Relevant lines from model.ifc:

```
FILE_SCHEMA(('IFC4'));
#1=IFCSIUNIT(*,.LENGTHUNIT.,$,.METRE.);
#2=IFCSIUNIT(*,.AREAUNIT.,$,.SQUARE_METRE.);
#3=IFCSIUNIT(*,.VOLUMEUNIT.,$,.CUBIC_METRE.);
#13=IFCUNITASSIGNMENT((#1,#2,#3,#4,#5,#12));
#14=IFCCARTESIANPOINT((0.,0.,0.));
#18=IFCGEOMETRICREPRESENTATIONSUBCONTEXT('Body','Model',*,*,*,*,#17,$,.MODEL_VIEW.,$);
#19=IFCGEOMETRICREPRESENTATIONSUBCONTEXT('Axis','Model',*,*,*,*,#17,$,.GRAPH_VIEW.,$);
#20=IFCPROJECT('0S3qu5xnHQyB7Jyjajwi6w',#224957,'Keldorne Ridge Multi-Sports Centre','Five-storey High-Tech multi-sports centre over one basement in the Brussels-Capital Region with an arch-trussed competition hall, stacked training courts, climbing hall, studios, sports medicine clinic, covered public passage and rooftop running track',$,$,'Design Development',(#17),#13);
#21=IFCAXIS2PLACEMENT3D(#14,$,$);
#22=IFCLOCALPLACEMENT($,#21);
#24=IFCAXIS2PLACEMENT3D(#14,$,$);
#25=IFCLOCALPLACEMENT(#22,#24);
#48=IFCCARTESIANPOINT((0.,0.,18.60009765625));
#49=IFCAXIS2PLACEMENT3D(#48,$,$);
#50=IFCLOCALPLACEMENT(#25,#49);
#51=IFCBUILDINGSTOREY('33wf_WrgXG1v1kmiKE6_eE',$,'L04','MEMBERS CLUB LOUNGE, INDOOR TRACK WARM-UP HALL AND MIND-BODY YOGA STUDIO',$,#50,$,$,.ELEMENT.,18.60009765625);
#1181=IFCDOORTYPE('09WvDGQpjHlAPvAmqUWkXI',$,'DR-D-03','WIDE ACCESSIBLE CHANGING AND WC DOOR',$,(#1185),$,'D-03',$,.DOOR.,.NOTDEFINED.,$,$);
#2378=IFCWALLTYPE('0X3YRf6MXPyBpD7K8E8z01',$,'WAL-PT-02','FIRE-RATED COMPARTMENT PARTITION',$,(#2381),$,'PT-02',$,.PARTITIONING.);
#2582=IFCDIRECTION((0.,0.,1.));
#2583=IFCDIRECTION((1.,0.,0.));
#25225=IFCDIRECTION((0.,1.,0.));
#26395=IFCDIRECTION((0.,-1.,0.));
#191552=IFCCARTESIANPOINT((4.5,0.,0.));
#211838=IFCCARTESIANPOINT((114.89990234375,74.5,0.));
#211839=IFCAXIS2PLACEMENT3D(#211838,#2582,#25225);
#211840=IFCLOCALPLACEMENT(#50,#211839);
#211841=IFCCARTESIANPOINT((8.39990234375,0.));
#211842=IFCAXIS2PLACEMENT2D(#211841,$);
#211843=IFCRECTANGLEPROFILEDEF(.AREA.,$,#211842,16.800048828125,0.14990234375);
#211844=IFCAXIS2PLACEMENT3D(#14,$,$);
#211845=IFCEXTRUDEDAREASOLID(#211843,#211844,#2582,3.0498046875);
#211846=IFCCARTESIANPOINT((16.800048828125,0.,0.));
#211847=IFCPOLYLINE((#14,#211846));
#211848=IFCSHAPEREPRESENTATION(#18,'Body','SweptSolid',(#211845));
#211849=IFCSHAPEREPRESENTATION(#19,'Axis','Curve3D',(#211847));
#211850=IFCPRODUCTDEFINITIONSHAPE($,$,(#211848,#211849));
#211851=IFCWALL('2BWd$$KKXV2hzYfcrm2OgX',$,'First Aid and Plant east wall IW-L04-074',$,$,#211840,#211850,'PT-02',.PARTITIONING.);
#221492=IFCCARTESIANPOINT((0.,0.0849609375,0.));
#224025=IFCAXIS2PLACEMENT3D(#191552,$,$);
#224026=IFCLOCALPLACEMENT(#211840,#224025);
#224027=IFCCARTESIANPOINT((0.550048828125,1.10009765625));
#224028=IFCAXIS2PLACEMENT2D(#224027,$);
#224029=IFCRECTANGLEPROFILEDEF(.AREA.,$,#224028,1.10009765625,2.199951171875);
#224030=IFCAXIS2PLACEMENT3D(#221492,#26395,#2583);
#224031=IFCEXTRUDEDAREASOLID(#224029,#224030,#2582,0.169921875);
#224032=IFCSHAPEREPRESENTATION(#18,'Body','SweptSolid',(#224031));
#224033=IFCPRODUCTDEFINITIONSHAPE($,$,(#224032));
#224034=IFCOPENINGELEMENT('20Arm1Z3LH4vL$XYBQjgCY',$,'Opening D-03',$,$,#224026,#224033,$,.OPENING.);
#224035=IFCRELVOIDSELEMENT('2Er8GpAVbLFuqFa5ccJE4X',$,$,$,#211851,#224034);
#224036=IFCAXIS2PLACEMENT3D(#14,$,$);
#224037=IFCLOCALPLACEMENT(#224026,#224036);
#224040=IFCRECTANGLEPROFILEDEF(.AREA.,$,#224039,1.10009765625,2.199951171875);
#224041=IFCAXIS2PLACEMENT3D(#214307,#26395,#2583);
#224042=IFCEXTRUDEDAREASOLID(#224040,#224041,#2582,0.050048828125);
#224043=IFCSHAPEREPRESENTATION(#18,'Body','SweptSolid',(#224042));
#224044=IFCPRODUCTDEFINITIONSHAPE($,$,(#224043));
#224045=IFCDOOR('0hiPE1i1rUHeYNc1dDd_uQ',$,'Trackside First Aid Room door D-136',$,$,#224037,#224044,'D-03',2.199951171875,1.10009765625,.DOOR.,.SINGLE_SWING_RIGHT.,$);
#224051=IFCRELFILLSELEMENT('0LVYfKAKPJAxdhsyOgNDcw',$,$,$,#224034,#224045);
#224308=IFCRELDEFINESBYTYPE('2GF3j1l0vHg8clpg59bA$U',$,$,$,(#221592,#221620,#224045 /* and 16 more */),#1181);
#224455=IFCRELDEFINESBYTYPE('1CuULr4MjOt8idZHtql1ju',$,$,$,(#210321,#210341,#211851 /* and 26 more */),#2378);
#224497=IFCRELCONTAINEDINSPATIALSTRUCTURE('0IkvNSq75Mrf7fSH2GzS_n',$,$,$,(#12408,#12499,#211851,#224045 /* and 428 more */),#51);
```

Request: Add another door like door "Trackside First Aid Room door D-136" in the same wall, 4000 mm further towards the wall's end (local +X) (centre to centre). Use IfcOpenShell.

```python
import ifcopenshell
import ifcopenshell.api.feature
import ifcopenshell.api.geometry
import ifcopenshell.api.root
import ifcopenshell.geom
import ifcopenshell.util.element
import ifcopenshell.util.placement
import ifcopenshell.util.shape

model = ifcopenshell.open("model.ifc")
settings = ifcopenshell.geom.settings()


def volume(element):
    """Net volume in cubic metres, openings subtracted."""
    shape = ifcopenshell.geom.create_shape(settings, element)
    return ifcopenshell.util.shape.get_volume(shape.geometry)


door = model.by_guid("0hiPE1i1rUHeYNc1dDd_uQ")
opening = door.FillsVoids[0].RelatingOpeningElement
wall = opening.VoidsElements[0].RelatingBuildingElement
before = volume(wall)
shift = ifcopenshell.util.placement.get_local_placement(wall.ObjectPlacement)[:3, 0] * 4.0

# copy_class copies the void relationship, type, container and properties, but no geometry.
new_opening = ifcopenshell.api.root.copy_class(model, product=opening)
new_opening.Representation = ifcopenshell.util.element.copy_deep(
    model, opening.Representation, exclude=["IfcGeometricRepresentationContext", "IfcRepresentationMap"]
)
new_door = ifcopenshell.api.root.copy_class(model, product=door)
new_door.Representation = ifcopenshell.util.element.copy_deep(
    model, door.Representation, exclude=["IfcGeometricRepresentationContext", "IfcRepresentationMap"]
)
new_door.Tag = None
ifcopenshell.api.feature.add_filling(model, opening=new_opening, element=new_door)

for old, new in ((opening, new_opening), (door, new_door)):
    matrix = ifcopenshell.util.placement.get_local_placement(old.ObjectPlacement)
    matrix[:3, 3] += shift
    ifcopenshell.api.geometry.edit_object_placement(model, product=new, matrix=matrix, is_si=False)

after = volume(wall)

print(f"wall volume {before:.3f} -> {after:.3f} m3")

model.write("model_updated.ifc")
```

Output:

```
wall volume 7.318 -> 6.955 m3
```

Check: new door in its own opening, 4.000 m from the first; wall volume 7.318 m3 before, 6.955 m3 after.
